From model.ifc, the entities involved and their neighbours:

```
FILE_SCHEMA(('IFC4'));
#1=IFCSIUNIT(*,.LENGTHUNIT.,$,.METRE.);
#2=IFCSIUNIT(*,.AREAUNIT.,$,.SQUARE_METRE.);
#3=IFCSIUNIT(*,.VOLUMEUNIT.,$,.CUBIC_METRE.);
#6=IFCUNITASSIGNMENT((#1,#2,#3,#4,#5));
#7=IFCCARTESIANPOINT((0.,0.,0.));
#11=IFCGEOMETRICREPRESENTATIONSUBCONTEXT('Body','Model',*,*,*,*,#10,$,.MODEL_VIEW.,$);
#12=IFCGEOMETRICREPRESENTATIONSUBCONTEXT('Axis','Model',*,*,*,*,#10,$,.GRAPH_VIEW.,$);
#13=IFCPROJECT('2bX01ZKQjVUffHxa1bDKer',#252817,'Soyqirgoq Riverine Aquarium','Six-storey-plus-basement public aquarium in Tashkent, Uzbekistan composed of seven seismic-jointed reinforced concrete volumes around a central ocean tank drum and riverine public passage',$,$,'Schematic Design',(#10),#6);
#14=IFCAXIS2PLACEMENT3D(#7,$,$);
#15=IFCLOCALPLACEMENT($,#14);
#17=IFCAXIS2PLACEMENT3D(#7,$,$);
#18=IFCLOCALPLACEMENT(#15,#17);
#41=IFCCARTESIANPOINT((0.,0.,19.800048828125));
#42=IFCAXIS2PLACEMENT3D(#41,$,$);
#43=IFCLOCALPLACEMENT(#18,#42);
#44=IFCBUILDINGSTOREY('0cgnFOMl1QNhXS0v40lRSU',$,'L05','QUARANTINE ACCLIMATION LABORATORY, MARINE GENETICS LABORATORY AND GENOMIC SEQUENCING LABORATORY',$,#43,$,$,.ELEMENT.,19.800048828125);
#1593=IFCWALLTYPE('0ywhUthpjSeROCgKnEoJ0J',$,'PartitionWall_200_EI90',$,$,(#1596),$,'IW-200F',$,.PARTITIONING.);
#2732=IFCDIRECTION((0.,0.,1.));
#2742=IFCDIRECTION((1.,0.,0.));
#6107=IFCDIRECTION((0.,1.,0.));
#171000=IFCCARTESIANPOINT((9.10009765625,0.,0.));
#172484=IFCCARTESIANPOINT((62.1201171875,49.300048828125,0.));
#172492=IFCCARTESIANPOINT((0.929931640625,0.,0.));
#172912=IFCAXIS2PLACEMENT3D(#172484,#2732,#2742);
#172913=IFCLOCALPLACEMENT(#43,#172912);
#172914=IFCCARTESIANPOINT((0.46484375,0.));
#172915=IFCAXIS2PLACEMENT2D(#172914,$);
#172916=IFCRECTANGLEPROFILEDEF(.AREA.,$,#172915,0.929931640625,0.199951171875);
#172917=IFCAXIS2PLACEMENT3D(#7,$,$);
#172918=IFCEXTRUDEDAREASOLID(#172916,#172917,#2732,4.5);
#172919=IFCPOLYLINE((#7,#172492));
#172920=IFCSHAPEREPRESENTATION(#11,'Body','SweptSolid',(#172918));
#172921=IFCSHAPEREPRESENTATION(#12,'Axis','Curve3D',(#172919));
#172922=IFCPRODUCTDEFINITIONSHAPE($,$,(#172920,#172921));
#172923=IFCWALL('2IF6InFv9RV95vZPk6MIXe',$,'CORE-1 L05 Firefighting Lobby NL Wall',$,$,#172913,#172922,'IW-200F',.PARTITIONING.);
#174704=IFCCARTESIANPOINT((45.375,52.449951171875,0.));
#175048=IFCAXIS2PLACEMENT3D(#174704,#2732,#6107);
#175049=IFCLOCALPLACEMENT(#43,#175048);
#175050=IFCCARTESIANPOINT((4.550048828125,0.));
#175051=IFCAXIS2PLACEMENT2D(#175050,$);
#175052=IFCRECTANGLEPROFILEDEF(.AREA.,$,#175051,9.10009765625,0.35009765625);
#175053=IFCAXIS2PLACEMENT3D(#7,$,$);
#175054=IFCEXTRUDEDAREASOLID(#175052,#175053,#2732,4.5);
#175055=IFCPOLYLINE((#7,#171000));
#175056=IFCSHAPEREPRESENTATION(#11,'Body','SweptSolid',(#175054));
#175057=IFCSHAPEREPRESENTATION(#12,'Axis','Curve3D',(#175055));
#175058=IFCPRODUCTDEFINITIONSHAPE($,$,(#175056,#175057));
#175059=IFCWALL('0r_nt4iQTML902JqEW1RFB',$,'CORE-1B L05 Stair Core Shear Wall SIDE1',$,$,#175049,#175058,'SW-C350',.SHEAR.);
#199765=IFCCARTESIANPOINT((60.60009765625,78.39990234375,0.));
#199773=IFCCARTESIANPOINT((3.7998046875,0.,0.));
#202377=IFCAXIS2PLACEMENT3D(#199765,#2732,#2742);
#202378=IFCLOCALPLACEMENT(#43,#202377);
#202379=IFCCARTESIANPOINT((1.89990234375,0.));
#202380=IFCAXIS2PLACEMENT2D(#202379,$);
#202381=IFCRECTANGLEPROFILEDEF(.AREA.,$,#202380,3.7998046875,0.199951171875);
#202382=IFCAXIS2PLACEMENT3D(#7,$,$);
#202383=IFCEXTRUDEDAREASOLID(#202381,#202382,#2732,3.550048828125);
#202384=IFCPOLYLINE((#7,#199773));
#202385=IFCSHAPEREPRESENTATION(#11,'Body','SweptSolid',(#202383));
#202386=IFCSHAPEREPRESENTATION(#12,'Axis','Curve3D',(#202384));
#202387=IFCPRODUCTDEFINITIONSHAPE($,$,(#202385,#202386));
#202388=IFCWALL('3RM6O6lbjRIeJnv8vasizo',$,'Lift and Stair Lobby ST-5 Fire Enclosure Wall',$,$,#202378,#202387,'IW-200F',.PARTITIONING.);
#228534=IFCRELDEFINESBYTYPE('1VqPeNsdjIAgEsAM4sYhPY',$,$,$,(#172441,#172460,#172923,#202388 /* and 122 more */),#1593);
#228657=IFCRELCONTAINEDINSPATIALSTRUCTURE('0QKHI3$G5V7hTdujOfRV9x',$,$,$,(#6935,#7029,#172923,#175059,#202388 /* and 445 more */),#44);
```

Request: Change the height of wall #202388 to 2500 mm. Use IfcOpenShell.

```python
import ifcopenshell
import ifcopenshell.geom
import ifcopenshell.util.representation
import ifcopenshell.util.shape

model = ifcopenshell.open("model.ifc")
settings = ifcopenshell.geom.settings()


def volume(element):
    """Net volume in cubic metres, openings subtracted."""
    shape = ifcopenshell.geom.create_shape(settings, element)
    return ifcopenshell.util.shape.get_volume(shape.geometry)


wall = model.by_guid("3RM6O6lbjRIeJnv8vasizo")
before = volume(wall)

body = ifcopenshell.util.representation.get_representation(wall, "Model", "Body")
solid = body.Items[0]
old_height = solid.Depth
solid.Depth = 2.5
after = volume(wall)

print(f"height {old_height:g} -> {solid.Depth:g}, volume {before:.3f} -> {after:.3f} m3")

model.write("model-out.ifc")
```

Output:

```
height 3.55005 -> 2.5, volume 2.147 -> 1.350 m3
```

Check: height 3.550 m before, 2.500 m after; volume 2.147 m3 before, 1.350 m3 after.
